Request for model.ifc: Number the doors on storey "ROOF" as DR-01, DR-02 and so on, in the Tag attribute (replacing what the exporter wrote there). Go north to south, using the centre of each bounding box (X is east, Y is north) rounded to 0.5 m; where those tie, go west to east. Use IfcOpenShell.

First a look at what the model holds.

```python
import ifcopenshell
import ifcopenshell.util.element
import ifcopenshell.util.placement

model = ifcopenshell.open("model.ifc")
print(model.schema)
storey = next(s for s in model.by_type("IfcBuildingStorey") if s.Name == "ROOF")
doors = [e for e in ifcopenshell.util.element.get_decomposition(storey) if e.is_a("IfcDoor")]
for e in sorted(doors, key=lambda e: e.id()):
    origin = ifcopenshell.util.placement.get_local_placement(e.ObjectPlacement)[:3, 3]
    print(e.id(), e.Tag, e.Name, origin.round(2) + 0.0, sep=" | ")
```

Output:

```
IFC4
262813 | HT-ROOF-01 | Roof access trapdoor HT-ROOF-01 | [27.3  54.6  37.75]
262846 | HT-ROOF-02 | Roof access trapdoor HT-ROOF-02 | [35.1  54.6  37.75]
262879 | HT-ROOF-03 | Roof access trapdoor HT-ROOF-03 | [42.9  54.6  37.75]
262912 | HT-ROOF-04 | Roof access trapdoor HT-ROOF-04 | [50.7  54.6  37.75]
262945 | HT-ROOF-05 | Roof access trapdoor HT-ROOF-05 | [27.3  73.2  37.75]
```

```python
import ifcopenshell
import ifcopenshell.geom
import ifcopenshell.util.element
import ifcopenshell.util.shape

model = ifcopenshell.open("model.ifc")
settings = ifcopenshell.geom.settings()
settings.set("use-world-coords", True)


def centre(element):
    shape = ifcopenshell.geom.create_shape(settings, element)
    return ifcopenshell.util.shape.get_bbox_centroid(shape.geometry)


storey = next(s for s in model.by_type("IfcBuildingStorey") if s.Name == "ROOF")
doors = [e for e in ifcopenshell.util.element.get_decomposition(storey) if e.is_a("IfcDoor")]

# Insertion points can sit at a corner or the storey origin, so sort by the geometry (in metres).
centres = {e: centre(e) for e in doors}
doors.sort(key=lambda e: (-round(centres[e][1] / 0.5), centres[e][0]))

for i, e in enumerate(doors, start=1):
    number = f"DR-{i:02d}"
    e.Tag = number
    print(e.id(), number)

model.write("model-out.ifc")
```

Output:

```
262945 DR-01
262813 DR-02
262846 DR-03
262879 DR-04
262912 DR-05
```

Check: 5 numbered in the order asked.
